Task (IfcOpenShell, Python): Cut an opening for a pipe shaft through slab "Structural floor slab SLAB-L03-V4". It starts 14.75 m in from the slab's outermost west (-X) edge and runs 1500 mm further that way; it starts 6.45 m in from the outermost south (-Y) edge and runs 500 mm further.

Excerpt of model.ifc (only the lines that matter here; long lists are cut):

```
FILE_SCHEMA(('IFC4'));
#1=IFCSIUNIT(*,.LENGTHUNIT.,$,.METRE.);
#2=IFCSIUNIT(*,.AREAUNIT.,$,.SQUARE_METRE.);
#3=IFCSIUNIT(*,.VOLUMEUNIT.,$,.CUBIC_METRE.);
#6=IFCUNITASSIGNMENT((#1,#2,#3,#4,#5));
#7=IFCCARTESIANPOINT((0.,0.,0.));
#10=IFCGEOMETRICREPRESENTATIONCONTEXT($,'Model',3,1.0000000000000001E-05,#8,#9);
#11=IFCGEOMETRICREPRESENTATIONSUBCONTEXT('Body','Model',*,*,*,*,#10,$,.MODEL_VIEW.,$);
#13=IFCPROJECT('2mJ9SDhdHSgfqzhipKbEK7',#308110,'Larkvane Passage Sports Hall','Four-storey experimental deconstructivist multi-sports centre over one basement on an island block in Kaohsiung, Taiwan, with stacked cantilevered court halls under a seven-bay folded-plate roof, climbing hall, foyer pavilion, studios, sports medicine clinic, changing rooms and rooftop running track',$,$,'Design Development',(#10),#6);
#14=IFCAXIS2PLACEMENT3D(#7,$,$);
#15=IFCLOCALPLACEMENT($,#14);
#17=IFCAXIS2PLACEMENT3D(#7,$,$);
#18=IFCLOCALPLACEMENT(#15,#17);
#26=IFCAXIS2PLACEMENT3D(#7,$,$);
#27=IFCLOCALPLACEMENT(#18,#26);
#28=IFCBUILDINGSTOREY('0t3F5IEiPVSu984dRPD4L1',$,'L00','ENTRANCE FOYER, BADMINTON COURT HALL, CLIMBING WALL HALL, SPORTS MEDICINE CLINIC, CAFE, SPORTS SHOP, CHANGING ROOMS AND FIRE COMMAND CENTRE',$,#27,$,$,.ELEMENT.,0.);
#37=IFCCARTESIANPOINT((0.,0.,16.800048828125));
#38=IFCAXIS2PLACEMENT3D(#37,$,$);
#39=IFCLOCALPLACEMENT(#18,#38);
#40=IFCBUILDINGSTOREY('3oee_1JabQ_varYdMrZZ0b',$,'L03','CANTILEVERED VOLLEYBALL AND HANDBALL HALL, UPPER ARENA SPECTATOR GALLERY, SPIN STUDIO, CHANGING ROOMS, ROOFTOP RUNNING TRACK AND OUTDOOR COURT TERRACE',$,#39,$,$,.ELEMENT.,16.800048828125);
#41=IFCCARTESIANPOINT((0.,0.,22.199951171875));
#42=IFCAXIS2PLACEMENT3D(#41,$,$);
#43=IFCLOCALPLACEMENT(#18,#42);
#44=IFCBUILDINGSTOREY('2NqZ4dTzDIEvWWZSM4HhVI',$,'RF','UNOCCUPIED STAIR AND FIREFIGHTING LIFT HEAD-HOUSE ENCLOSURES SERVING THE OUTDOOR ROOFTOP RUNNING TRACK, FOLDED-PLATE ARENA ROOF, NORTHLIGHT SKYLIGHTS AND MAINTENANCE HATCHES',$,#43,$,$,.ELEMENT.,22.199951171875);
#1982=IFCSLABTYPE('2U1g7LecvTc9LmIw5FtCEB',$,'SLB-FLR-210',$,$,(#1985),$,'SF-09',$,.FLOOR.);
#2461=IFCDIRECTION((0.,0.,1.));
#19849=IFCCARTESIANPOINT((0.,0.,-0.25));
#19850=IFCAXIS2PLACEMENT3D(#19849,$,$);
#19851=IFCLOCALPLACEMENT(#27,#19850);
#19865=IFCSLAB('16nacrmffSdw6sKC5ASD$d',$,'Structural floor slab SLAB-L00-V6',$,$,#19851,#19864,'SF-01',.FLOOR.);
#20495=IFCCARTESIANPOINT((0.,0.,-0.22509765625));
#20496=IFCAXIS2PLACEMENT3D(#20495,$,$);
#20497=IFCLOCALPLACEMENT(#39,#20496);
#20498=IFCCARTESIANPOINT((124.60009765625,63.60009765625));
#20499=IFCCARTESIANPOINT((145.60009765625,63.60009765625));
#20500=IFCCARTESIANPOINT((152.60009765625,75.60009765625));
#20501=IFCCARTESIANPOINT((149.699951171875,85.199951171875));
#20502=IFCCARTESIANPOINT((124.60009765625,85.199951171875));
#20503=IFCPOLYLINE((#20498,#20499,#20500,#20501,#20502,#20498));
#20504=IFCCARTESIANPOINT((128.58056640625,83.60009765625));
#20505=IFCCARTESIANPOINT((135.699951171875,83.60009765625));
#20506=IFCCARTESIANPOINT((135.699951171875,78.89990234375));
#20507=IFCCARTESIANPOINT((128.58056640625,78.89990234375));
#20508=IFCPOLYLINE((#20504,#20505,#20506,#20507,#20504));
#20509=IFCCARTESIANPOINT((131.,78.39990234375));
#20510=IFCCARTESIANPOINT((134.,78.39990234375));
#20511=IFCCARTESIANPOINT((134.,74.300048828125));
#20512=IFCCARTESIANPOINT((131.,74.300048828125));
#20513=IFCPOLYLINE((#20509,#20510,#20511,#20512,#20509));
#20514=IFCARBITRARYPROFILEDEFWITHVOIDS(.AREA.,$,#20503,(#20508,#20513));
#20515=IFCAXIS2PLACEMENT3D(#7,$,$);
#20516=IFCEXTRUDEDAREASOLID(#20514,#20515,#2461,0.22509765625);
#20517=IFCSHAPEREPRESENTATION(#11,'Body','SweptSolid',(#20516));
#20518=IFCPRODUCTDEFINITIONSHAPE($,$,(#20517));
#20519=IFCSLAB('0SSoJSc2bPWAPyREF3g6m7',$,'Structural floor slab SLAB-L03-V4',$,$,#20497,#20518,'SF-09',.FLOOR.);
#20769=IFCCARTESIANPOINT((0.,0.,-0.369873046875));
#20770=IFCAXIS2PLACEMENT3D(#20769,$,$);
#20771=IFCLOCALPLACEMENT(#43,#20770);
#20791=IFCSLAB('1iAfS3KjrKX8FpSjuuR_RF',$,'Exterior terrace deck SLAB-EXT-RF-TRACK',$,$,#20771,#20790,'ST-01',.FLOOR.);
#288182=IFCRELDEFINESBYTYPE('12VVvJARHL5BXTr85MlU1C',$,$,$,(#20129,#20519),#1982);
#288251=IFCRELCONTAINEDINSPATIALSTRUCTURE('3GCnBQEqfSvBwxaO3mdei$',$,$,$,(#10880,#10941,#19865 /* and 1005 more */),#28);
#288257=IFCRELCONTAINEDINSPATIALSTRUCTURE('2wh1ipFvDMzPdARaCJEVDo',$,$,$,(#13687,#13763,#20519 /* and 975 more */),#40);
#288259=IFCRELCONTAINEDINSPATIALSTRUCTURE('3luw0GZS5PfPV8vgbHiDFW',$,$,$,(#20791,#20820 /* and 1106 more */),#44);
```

```python
import numpy as np
import ifcopenshell
import ifcopenshell.api.feature
import ifcopenshell.api.geometry
import ifcopenshell.api.root
import ifcopenshell.geom
import ifcopenshell.util.placement
import ifcopenshell.util.representation
import ifcopenshell.util.shape
import ifcopenshell.util.unit

model = ifcopenshell.open("model.ifc")
unit_scale = ifcopenshell.util.unit.calculate_unit_scale(model)
settings = ifcopenshell.geom.settings()


def volume(element):
    """Net volume in cubic metres, openings subtracted."""
    shape = ifcopenshell.geom.create_shape(settings, element)
    return ifcopenshell.util.shape.get_volume(shape.geometry)


slab = model.by_guid("0SSoJSc2bPWAPyREF3g6m7")
before = volume(slab)

# Extent in the slab's own axes, in metres. The edges named are its -X and -Y sides.
slab_shape = ifcopenshell.geom.create_shape(settings, slab)
vertices = ifcopenshell.util.shape.get_vertices(slab_shape.geometry)
x_min, y_min, bottom = vertices.min(axis=0)
top = vertices[:, 2].max()

opening = ifcopenshell.api.root.create_entity(model, ifc_class="IfcOpeningElement", name="Pipe shaft opening", predefined_type="OPENING")
context = ifcopenshell.util.representation.get_context(model, "Model", "Body", "MODEL_VIEW")
width, depth = 1.5, 0.5
outline = [(0.0, 0.0), (width, 0.0), (width, depth), (0.0, depth), (0.0, 0.0)]
# Overshoot both faces by 50 mm so the cut is clean.
shape = ifcopenshell.api.geometry.add_slab_representation(
    model, context=context, depth=top - bottom + 0.1, polyline=outline
)
ifcopenshell.api.geometry.assign_representation(model, product=opening, representation=shape)

matrix = ifcopenshell.util.placement.get_local_placement(slab.ObjectPlacement)
matrix[:, 3] = matrix @ np.append(np.array([x_min + 14.75, y_min + 6.45, bottom - 0.05]) / unit_scale, 1.0)
ifcopenshell.api.geometry.edit_object_placement(model, product=opening, matrix=matrix, is_si=False)
ifcopenshell.api.feature.add_feature(model, feature=opening, element=slab)

after = volume(slab)

print(f"slab volume {before:.3f} -> {after:.3f} m3")

model.write("model-out.ifc")
```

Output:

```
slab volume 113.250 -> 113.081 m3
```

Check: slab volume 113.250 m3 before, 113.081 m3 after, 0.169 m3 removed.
